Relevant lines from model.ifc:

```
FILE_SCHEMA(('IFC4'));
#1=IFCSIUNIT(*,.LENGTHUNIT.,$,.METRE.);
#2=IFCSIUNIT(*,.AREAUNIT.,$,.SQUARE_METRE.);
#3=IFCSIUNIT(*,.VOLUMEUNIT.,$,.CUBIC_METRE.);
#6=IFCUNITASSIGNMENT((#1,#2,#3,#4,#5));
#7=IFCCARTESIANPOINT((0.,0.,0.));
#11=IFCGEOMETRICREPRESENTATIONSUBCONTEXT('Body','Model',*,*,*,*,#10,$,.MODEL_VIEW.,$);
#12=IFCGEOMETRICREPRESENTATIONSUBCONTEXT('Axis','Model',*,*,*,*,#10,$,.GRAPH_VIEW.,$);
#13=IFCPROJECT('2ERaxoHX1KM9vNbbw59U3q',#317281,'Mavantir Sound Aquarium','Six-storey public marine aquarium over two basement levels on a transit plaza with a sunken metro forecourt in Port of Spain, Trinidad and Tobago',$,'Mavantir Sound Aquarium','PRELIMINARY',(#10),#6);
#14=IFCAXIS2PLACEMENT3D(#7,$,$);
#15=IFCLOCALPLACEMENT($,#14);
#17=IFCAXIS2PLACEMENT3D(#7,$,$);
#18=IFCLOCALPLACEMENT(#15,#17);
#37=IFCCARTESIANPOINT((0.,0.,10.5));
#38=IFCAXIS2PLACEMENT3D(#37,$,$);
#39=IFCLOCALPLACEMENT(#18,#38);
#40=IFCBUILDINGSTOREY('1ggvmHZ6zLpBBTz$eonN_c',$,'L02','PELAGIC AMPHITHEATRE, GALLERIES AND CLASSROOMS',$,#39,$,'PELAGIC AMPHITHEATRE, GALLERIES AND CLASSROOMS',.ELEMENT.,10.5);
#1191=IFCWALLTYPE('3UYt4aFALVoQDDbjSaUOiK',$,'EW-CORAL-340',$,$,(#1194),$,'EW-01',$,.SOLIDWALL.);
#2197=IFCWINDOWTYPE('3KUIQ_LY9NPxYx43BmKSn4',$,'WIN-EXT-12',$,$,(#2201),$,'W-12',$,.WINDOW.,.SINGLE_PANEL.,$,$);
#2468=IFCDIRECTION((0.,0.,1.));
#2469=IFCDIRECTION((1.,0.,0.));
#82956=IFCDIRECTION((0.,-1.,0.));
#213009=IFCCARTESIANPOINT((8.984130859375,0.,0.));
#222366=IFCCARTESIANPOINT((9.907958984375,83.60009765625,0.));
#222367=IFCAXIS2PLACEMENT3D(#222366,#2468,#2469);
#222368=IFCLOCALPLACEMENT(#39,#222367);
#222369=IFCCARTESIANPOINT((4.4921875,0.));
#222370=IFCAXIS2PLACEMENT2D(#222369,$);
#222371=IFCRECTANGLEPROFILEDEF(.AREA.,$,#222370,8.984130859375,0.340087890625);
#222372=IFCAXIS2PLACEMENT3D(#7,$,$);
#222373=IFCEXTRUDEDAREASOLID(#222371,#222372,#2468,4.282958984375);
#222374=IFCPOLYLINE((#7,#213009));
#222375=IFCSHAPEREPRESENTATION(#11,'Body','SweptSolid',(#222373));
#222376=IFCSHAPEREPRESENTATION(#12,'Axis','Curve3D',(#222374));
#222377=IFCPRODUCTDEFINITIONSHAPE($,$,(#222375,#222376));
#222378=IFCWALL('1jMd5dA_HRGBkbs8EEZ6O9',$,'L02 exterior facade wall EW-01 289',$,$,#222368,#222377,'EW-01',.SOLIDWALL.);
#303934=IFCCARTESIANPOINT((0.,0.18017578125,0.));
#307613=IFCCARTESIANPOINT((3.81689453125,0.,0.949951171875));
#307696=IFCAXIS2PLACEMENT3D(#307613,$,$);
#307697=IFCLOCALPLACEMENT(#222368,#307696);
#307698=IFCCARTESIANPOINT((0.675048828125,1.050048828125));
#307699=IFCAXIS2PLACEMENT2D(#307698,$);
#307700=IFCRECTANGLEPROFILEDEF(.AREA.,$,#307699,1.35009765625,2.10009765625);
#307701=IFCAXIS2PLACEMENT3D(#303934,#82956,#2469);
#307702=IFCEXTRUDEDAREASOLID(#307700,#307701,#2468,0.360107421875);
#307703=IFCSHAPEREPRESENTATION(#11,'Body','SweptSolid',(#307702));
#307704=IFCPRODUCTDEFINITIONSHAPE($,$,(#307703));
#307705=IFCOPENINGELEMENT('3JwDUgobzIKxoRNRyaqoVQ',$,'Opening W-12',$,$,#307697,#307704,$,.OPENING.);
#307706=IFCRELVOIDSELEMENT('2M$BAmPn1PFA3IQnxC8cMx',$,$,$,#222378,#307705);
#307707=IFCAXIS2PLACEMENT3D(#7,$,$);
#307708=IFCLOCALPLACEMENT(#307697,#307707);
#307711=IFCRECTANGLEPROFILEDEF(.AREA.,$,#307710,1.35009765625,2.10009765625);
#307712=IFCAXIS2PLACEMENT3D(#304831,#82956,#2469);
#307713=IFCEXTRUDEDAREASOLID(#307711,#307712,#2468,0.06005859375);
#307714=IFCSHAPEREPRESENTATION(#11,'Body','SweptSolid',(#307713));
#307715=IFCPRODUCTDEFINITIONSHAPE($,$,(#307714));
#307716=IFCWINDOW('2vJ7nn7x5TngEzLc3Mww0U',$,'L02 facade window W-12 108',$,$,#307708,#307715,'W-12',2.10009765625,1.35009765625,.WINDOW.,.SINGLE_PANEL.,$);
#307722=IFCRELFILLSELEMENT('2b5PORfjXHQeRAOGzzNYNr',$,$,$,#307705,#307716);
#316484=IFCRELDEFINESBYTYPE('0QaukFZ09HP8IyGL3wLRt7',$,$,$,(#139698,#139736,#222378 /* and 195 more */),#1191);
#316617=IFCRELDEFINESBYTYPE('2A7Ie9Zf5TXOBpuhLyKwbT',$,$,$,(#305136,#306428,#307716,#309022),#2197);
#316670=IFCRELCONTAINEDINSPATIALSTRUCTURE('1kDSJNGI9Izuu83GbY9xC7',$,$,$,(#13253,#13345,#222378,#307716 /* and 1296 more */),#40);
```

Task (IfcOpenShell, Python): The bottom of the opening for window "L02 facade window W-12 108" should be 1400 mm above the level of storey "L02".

```python
import numpy as np
import ifcopenshell
import ifcopenshell.api.geometry
import ifcopenshell.geom
import ifcopenshell.util.element
import ifcopenshell.util.placement
import ifcopenshell.util.shape
import ifcopenshell.util.unit

model = ifcopenshell.open("model.ifc")
unit_scale = ifcopenshell.util.unit.calculate_unit_scale(model)

window = model.by_guid("2vJ7nn7x5TngEzLc3Mww0U")
opening = window.FillsVoids[0].RelatingOpeningElement
storey = ifcopenshell.util.element.get_container(window, ifc_class="IfcBuildingStorey")
level = ifcopenshell.util.placement.get_local_placement(storey.ObjectPlacement)[2, 3]

# The opening's origin need not be at the sill, so measure its lowest point.
shape = ifcopenshell.geom.create_shape(ifcopenshell.geom.settings(), opening)
bottom = ifcopenshell.util.shape.get_shape_bottom_elevation(shape, shape.geometry) / unit_scale
dz = level + 1.4 - bottom

shift = np.array([0.0, 0.0, dz])
# The window is placed relative to its opening, so it follows when the opening moves.
matrix = ifcopenshell.util.placement.get_local_placement(opening.ObjectPlacement)
matrix[:3, 3] += shift
ifcopenshell.api.geometry.edit_object_placement(
    model, product=opening, matrix=matrix, is_si=False, should_transform_children=True
)

print(f"moved by {dz * unit_scale:+.3f} m")

model.write("model_updated.ifc")
```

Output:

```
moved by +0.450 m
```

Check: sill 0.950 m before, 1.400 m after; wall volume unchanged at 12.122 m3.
